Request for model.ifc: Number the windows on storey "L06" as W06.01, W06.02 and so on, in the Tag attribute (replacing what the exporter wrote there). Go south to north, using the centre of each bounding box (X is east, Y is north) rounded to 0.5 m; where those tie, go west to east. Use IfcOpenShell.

First a look at what the model holds.

```python
import ifcopenshell
import ifcopenshell.util.element
import ifcopenshell.util.placement

model = ifcopenshell.open("model.ifc")
print(model.schema)
storey = next(s for s in model.by_type("IfcBuildingStorey") if s.Name == "L06")
windows = [e for e in ifcopenshell.util.element.get_decomposition(storey) if e.is_a("IfcWindow")]
for e in sorted(windows, key=lambda e: e.id()):
    origin = ifcopenshell.util.placement.get_local_placement(e.ObjectPlacement)[:3, 3]
    print(e.id(), e.Tag, e.Name, origin.round(2) + 0.0, sep=" | ")
```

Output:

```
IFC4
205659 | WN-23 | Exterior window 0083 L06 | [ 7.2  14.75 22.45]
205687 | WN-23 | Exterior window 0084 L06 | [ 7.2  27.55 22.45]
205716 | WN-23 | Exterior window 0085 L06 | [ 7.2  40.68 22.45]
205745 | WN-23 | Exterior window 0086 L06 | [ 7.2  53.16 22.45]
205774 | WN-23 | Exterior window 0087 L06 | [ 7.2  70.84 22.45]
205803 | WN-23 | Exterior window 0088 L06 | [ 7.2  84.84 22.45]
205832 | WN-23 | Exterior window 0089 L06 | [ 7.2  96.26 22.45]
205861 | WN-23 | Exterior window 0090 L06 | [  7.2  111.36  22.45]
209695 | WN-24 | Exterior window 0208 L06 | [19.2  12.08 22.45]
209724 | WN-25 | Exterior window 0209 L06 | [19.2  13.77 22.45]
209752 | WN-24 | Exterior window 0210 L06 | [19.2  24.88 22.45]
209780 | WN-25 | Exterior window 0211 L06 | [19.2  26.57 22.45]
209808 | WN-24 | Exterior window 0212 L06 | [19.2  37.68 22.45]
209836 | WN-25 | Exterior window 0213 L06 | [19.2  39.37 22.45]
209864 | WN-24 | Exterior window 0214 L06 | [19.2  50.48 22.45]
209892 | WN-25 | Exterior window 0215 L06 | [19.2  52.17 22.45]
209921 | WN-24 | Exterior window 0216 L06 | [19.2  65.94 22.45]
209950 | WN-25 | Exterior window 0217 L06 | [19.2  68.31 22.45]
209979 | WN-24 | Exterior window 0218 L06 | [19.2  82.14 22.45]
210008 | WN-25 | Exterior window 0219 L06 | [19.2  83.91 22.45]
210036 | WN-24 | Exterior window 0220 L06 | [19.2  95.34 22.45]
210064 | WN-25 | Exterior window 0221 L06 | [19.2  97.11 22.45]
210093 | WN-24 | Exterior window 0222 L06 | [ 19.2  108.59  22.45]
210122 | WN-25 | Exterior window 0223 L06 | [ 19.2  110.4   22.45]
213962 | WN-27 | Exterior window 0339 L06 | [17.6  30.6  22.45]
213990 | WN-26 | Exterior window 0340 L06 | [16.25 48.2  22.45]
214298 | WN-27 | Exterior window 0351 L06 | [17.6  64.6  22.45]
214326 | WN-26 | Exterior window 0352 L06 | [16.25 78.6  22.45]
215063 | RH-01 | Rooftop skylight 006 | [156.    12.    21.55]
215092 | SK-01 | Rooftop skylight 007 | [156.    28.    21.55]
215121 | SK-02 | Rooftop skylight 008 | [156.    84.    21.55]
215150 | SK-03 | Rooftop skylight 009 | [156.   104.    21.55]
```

```python
import ifcopenshell
import ifcopenshell.geom
import ifcopenshell.util.element
import ifcopenshell.util.shape

model = ifcopenshell.open("model.ifc")
settings = ifcopenshell.geom.settings()
settings.set("use-world-coords", True)


def centre(element):
    shape = ifcopenshell.geom.create_shape(settings, element)
    return ifcopenshell.util.shape.get_bbox_centroid(shape.geometry)


storey = next(s for s in model.by_type("IfcBuildingStorey") if s.Name == "L06")
windows = [e for e in ifcopenshell.util.element.get_decomposition(storey) if e.is_a("IfcWindow")]

# Insertion points can sit at a corner or the storey origin, so sort by the geometry (in metres).
centres = {e: centre(e) for e in windows}
windows.sort(key=lambda e: (round(centres[e][1] / 0.5), centres[e][0]))

for i, e in enumerate(windows, start=1):
    number = f"W06.{i:02d}"
    e.Tag = number
    print(e.id(), number)

model.write("model_rev.ifc")
```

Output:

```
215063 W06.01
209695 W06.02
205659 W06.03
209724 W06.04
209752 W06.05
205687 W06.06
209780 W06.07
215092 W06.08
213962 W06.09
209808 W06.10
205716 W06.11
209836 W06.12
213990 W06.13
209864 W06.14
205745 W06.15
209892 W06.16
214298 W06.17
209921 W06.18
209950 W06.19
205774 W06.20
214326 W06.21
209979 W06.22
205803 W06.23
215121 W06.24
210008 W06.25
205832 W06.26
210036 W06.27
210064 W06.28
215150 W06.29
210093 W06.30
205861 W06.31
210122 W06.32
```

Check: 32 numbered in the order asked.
